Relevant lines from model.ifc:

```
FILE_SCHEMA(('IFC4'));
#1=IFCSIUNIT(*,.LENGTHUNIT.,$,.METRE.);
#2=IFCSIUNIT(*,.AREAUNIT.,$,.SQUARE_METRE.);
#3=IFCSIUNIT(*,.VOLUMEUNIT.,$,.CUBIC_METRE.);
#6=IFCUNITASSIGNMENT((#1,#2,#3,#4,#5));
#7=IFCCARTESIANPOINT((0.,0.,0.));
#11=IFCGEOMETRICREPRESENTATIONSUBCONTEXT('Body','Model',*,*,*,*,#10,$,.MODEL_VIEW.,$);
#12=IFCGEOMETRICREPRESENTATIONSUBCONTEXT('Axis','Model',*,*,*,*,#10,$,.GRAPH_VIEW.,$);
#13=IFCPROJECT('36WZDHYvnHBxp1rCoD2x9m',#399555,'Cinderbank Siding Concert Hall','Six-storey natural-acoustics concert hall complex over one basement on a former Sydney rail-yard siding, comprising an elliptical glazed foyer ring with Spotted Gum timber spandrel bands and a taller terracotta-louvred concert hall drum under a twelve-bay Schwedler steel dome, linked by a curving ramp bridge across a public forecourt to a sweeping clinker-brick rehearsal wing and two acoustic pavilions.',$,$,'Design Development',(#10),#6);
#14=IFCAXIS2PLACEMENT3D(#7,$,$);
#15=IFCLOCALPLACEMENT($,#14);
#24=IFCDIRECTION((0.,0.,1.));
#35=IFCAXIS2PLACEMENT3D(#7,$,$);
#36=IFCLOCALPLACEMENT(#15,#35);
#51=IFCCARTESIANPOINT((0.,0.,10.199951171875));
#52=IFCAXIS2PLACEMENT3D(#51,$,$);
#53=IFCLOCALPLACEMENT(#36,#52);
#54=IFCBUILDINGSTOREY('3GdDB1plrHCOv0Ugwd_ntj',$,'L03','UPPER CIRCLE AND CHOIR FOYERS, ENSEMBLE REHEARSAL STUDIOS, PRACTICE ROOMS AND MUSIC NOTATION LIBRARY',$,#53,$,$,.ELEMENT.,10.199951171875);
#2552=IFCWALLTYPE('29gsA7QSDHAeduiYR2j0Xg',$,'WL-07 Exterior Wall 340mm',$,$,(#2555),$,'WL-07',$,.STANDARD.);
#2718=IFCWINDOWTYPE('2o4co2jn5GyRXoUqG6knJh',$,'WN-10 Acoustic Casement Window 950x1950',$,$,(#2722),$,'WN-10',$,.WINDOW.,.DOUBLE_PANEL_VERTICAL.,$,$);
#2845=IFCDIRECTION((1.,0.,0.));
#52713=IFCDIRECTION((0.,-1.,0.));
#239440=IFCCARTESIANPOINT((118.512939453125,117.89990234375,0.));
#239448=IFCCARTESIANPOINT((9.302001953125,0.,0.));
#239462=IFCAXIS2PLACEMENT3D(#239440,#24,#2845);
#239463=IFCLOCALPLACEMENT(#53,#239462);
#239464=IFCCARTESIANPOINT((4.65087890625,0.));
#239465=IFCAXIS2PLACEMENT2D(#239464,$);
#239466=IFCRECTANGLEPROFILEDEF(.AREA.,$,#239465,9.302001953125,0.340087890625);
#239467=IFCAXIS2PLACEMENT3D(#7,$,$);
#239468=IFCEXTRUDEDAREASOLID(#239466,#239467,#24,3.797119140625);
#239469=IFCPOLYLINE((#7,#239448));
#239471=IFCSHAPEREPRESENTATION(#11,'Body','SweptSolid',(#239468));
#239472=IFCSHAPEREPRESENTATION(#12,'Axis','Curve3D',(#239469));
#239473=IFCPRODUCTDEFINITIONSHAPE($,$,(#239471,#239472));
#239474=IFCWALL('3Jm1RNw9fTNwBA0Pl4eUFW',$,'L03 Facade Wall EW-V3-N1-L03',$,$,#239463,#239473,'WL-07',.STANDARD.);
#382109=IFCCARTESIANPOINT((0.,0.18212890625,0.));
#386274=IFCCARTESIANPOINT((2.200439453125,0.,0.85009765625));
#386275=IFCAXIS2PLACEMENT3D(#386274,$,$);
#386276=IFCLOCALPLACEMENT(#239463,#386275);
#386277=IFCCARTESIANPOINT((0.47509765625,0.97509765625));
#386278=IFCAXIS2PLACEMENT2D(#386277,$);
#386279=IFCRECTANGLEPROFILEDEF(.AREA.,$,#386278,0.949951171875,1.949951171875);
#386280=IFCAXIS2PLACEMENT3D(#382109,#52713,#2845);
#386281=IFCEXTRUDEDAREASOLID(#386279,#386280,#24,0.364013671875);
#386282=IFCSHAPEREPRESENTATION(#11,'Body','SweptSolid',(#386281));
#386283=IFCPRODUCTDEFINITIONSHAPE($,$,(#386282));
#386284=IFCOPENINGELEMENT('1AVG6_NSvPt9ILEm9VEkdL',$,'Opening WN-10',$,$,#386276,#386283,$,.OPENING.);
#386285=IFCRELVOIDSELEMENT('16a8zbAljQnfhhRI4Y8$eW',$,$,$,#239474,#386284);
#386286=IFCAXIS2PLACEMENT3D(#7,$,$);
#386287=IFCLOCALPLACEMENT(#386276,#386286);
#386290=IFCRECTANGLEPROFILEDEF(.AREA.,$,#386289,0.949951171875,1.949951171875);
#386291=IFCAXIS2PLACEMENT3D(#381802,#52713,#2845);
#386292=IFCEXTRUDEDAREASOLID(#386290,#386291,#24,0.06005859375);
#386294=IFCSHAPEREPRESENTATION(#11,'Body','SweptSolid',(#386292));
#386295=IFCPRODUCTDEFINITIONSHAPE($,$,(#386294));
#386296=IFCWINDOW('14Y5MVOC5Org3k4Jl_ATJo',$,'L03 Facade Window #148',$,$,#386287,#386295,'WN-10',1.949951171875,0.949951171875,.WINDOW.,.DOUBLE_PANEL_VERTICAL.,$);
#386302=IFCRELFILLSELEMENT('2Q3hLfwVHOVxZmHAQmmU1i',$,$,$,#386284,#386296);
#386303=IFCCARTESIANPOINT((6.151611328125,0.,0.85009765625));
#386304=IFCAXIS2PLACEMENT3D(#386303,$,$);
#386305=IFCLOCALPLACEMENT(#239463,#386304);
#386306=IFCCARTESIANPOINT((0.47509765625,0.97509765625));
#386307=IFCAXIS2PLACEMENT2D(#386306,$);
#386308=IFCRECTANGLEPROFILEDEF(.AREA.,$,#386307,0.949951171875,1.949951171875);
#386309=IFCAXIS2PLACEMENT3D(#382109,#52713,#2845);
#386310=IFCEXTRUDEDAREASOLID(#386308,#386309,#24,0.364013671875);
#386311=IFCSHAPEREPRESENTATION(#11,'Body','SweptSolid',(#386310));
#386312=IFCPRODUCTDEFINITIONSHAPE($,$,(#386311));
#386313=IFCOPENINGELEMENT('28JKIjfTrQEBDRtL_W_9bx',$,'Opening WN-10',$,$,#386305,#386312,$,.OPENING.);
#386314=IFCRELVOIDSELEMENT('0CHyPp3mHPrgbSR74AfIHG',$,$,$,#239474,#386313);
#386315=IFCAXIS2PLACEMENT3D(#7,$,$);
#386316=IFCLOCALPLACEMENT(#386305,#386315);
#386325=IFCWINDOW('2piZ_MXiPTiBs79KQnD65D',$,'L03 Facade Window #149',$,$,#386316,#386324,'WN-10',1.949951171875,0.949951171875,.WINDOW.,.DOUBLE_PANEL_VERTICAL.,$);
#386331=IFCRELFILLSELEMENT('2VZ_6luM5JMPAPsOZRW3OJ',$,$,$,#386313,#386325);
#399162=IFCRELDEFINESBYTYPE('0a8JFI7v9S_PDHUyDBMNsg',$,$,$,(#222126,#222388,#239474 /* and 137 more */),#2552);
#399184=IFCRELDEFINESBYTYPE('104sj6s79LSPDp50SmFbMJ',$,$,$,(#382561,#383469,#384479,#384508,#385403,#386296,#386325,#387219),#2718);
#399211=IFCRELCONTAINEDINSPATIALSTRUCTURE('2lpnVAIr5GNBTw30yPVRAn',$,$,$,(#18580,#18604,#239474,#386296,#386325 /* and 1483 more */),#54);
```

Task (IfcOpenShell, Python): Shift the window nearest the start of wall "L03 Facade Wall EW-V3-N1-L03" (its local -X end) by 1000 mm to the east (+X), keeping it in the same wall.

```python
import ifcopenshell
import ifcopenshell.api.geometry
import ifcopenshell.util.placement
import ifcopenshell.util.unit

model = ifcopenshell.open("model.ifc")
unit_scale = ifcopenshell.util.unit.calculate_unit_scale(model)

window = model.by_guid("14Y5MVOC5Org3k4Jl_ATJo")
opening = window.FillsVoids[0].RelatingOpeningElement
wall = opening.VoidsElements[0].RelatingBuildingElement

wall_matrix = ifcopenshell.util.placement.get_local_placement(wall.ObjectPlacement)
shift = wall_matrix[:3, 0] * 1 / unit_scale
before = ifcopenshell.util.placement.get_local_placement(window.ObjectPlacement)[:3, 3].copy()

# The window is placed relative to its opening, so it follows when the opening moves.
matrix = ifcopenshell.util.placement.get_local_placement(opening.ObjectPlacement)
matrix[:3, 3] += shift
ifcopenshell.api.geometry.edit_object_placement(
    model, product=opening, matrix=matrix, is_si=False, should_transform_children=True
)

after = ifcopenshell.util.placement.get_local_placement(window.ObjectPlacement)[:3, 3]
print("window moved by", (after - before).round(3) + 0.0)

model.write("model_updated.ifc")
```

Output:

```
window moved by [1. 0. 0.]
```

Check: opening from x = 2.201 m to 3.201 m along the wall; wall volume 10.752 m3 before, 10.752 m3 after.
